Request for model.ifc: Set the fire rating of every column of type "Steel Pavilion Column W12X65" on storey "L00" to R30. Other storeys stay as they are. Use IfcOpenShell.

First a look at what the model holds.

```python
import ifcopenshell
import ifcopenshell.util.element

model = ifcopenshell.open("model.ifc")
print(model.schema)
storey = next(s for s in model.by_type("IfcBuildingStorey") if s.Name == "L00")
columns = [e for e in ifcopenshell.util.element.get_decomposition(storey) if e.is_a("IfcColumn")]
seen = {}
for e in columns:
    element_type = ifcopenshell.util.element.get_type(e)
    key = (element_type.Name if element_type != e and element_type else None, ifcopenshell.util.element.get_pset(e, "Pset_ColumnCommon", "FireRating"))
    seen[key] = seen.get(key, 0) + 1
for (name, value), count in sorted(seen.items(), key=str):
    print(count, "x", name, "|", value)
```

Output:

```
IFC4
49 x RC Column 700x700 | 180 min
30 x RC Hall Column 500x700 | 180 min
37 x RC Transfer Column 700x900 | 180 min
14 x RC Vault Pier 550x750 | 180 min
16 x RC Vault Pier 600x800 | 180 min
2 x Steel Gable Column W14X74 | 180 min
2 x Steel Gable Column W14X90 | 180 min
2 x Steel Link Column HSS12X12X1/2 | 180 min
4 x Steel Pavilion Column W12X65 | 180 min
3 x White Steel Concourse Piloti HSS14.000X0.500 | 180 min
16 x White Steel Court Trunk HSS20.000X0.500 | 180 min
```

```python
import ifcopenshell
import ifcopenshell.api.pset
import ifcopenshell.util.element

model = ifcopenshell.open("model.ifc")

storey = next(s for s in model.by_type("IfcBuildingStorey") if s.Name == "L00")
columns = [e for e in ifcopenshell.util.element.get_decomposition(storey) if e.is_a("IfcColumn")]

count = 0
for e in columns:
    element_type = ifcopenshell.util.element.get_type(e)
    if element_type in (None, e) or element_type.Name != "Steel Pavilion Column W12X65":
        continue
    # add_pset returns the element's existing set when there is one.
    pset = ifcopenshell.api.pset.add_pset(model, product=e, name="Pset_ColumnCommon")
    ifcopenshell.api.pset.edit_pset(model, pset=pset, properties={"FireRating": "R30"})
    count += 1

print(count, "columns updated")

model.write("model-out.ifc")
```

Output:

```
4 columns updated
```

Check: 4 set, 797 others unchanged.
